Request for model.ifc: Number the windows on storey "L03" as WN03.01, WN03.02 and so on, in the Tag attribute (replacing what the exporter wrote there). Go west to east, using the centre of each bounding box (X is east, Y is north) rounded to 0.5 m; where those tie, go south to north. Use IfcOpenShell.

First a look at what the model holds.

```python
import ifcopenshell
import ifcopenshell.util.element
import ifcopenshell.util.placement

model = ifcopenshell.open("model.ifc")
print(model.schema)
storey = next(s for s in model.by_type("IfcBuildingStorey") if s.Name == "L03")
windows = [e for e in ifcopenshell.util.element.get_decomposition(storey) if e.is_a("IfcWindow")]
for e in sorted(windows, key=lambda e: e.id()):
    origin = ifcopenshell.util.placement.get_local_placement(e.ObjectPlacement)[:3, 3]
    print(e.id(), e.Tag, e.Name, origin.round(2) + 0.0, sep=" | ")
```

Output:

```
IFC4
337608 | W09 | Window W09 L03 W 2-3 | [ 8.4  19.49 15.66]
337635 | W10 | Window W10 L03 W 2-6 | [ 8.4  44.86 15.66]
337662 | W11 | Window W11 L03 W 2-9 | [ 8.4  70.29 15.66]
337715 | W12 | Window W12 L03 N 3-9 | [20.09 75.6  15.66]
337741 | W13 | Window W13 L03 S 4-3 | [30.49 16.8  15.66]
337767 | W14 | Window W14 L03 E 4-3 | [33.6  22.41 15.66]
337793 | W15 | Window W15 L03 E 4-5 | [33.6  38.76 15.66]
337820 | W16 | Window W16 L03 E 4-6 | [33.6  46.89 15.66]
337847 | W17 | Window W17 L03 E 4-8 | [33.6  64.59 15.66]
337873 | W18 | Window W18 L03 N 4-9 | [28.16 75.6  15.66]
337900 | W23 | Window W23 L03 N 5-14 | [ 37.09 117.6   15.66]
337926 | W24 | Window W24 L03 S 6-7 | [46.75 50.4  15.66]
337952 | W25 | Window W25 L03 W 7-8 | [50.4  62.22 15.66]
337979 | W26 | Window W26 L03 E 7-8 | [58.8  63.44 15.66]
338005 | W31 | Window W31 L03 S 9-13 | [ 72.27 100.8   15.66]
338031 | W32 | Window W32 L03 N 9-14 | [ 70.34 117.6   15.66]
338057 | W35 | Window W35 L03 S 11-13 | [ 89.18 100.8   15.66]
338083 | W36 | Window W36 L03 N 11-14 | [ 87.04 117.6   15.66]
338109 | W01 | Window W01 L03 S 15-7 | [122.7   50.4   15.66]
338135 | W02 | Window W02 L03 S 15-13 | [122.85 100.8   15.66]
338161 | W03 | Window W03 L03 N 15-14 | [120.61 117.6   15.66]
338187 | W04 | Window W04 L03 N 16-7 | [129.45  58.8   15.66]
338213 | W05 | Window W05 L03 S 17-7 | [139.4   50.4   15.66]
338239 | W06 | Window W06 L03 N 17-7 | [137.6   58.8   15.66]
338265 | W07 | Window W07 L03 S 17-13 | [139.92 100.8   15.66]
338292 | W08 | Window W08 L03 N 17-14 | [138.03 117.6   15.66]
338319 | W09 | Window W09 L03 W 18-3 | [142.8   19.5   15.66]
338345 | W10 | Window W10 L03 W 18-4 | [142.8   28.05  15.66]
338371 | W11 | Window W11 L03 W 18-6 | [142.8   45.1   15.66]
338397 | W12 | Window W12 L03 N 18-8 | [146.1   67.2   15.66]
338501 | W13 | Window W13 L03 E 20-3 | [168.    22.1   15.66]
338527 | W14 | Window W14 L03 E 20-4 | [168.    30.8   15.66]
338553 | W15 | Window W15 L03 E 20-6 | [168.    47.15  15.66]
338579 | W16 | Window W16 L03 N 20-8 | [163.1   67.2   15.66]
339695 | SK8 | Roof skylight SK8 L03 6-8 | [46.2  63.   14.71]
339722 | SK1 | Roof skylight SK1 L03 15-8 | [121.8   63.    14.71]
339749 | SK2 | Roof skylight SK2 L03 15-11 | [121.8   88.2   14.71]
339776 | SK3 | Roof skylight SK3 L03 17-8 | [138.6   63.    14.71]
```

```python
import ifcopenshell
import ifcopenshell.geom
import ifcopenshell.util.element
import ifcopenshell.util.shape

model = ifcopenshell.open("model.ifc")
settings = ifcopenshell.geom.settings()
settings.set("use-world-coords", True)


def centre(element):
    shape = ifcopenshell.geom.create_shape(settings, element)
    return ifcopenshell.util.shape.get_bbox_centroid(shape.geometry)


storey = next(s for s in model.by_type("IfcBuildingStorey") if s.Name == "L03")
windows = [e for e in ifcopenshell.util.element.get_decomposition(storey) if e.is_a("IfcWindow")]

# Insertion points can sit at a corner or the storey origin, so sort by the geometry (in metres).
centres = {e: centre(e) for e in windows}
windows.sort(key=lambda e: (round(centres[e][0] / 0.5), centres[e][1]))

for i, e in enumerate(windows, start=1):
    number = f"WN03.{i:02d}"
    e.Tag = number
    print(e.id(), number)

model.write("model-out.ifc")
```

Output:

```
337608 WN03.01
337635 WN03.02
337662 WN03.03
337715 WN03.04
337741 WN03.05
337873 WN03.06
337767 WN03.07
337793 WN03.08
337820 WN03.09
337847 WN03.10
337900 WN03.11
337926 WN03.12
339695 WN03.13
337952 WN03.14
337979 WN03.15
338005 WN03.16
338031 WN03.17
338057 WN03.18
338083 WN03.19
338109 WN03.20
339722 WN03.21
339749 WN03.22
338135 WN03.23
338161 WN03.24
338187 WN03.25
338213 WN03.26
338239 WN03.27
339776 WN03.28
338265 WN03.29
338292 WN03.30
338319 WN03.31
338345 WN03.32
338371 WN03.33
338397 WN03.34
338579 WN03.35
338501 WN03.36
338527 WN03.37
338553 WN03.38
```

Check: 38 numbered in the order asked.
